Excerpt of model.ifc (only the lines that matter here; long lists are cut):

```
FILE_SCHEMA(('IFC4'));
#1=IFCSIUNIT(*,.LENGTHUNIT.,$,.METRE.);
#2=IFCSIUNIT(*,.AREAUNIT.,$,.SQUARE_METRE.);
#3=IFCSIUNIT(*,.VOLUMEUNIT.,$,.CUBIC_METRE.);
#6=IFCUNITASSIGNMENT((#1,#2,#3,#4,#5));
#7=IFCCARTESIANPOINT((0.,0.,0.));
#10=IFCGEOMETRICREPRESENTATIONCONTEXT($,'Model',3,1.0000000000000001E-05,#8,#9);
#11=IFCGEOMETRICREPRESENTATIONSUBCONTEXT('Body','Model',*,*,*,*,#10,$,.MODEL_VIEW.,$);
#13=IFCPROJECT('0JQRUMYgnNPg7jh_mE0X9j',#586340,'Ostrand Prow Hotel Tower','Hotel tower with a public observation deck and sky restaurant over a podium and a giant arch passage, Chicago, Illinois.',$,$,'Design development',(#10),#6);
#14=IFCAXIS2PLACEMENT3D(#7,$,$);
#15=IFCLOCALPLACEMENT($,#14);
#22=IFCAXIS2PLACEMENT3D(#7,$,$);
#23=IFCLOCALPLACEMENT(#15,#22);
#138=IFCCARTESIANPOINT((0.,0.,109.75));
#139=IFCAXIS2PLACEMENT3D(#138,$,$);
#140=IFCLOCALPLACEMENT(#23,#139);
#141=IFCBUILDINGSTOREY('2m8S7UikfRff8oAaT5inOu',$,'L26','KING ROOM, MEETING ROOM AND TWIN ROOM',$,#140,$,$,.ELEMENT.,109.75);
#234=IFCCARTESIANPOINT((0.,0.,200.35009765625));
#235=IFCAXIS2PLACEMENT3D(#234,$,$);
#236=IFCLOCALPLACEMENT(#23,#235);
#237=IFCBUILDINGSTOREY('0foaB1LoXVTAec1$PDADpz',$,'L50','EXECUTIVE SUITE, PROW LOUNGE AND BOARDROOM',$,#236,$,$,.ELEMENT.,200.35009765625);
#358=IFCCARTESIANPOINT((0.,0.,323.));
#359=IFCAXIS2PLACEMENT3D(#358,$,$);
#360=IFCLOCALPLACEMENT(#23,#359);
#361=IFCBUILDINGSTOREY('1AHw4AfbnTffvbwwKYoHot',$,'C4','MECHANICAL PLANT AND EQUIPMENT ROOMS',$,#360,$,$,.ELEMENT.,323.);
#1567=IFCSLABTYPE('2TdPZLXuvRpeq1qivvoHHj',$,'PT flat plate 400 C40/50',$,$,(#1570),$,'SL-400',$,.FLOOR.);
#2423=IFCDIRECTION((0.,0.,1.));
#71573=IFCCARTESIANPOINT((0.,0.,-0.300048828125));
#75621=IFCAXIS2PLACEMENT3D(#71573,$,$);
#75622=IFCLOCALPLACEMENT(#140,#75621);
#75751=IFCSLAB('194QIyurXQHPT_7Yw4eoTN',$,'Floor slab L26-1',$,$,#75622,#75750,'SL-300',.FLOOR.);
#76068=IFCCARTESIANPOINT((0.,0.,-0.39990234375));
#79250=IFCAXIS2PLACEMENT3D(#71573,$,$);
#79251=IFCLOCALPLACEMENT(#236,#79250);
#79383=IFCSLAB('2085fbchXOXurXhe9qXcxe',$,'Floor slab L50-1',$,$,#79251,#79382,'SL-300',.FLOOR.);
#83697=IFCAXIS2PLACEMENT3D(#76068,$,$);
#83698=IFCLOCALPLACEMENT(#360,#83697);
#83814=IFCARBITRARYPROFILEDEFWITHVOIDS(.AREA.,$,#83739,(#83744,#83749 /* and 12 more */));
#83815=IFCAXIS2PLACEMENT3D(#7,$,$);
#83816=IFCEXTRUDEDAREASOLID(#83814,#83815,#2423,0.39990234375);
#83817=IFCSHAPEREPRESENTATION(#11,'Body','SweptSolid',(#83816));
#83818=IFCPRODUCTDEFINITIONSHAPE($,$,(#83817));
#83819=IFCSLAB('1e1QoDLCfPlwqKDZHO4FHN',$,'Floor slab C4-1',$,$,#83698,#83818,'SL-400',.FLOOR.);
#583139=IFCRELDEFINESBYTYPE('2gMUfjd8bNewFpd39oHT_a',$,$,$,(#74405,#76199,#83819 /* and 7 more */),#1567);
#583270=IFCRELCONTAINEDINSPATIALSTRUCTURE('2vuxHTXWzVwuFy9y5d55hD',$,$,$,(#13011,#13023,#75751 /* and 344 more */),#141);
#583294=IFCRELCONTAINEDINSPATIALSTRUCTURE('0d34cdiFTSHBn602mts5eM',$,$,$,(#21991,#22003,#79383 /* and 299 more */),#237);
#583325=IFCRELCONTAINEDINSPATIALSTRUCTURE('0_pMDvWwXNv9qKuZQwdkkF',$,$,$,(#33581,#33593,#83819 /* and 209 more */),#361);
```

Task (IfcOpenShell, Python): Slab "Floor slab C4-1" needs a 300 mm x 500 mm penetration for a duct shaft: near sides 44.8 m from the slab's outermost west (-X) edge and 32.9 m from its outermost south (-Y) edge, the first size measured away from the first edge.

```python
import numpy as np
import ifcopenshell
import ifcopenshell.api.feature
import ifcopenshell.api.geometry
import ifcopenshell.api.root
import ifcopenshell.geom
import ifcopenshell.util.placement
import ifcopenshell.util.representation
import ifcopenshell.util.shape
import ifcopenshell.util.unit

model = ifcopenshell.open("model.ifc")
unit_scale = ifcopenshell.util.unit.calculate_unit_scale(model)
settings = ifcopenshell.geom.settings()


def volume(element):
    """Net volume in cubic metres, openings subtracted."""
    shape = ifcopenshell.geom.create_shape(settings, element)
    return ifcopenshell.util.shape.get_volume(shape.geometry)


slab = model.by_guid("1e1QoDLCfPlwqKDZHO4FHN")
before = volume(slab)

# Extent in the slab's own axes, in metres. The edges named are its -X and -Y sides.
slab_shape = ifcopenshell.geom.create_shape(settings, slab)
vertices = ifcopenshell.util.shape.get_vertices(slab_shape.geometry)
x_min, y_min, bottom = vertices.min(axis=0)
top = vertices[:, 2].max()

opening = ifcopenshell.api.root.create_entity(model, ifc_class="IfcOpeningElement", name="Duct shaft opening", predefined_type="OPENING")
context = ifcopenshell.util.representation.get_context(model, "Model", "Body", "MODEL_VIEW")
width, depth = 0.3, 0.5
outline = [(0.0, 0.0), (width, 0.0), (width, depth), (0.0, depth), (0.0, 0.0)]
# Overshoot both faces by 50 mm so the cut is clean.
shape = ifcopenshell.api.geometry.add_slab_representation(
    model, context=context, depth=top - bottom + 0.1, polyline=outline
)
ifcopenshell.api.geometry.assign_representation(model, product=opening, representation=shape)

matrix = ifcopenshell.util.placement.get_local_placement(slab.ObjectPlacement)
matrix[:, 3] = matrix @ np.append(np.array([x_min + 44.8, y_min + 32.9, bottom - 0.05]) / unit_scale, 1.0)
ifcopenshell.api.geometry.edit_object_placement(model, product=opening, matrix=matrix, is_si=False)
ifcopenshell.api.feature.add_feature(model, feature=opening, element=slab)

after = volume(slab)

print(f"slab volume {before:.3f} -> {after:.3f} m3")

model.write("model_edited.ifc")
```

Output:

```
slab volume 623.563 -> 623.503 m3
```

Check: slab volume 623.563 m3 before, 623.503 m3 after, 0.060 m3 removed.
